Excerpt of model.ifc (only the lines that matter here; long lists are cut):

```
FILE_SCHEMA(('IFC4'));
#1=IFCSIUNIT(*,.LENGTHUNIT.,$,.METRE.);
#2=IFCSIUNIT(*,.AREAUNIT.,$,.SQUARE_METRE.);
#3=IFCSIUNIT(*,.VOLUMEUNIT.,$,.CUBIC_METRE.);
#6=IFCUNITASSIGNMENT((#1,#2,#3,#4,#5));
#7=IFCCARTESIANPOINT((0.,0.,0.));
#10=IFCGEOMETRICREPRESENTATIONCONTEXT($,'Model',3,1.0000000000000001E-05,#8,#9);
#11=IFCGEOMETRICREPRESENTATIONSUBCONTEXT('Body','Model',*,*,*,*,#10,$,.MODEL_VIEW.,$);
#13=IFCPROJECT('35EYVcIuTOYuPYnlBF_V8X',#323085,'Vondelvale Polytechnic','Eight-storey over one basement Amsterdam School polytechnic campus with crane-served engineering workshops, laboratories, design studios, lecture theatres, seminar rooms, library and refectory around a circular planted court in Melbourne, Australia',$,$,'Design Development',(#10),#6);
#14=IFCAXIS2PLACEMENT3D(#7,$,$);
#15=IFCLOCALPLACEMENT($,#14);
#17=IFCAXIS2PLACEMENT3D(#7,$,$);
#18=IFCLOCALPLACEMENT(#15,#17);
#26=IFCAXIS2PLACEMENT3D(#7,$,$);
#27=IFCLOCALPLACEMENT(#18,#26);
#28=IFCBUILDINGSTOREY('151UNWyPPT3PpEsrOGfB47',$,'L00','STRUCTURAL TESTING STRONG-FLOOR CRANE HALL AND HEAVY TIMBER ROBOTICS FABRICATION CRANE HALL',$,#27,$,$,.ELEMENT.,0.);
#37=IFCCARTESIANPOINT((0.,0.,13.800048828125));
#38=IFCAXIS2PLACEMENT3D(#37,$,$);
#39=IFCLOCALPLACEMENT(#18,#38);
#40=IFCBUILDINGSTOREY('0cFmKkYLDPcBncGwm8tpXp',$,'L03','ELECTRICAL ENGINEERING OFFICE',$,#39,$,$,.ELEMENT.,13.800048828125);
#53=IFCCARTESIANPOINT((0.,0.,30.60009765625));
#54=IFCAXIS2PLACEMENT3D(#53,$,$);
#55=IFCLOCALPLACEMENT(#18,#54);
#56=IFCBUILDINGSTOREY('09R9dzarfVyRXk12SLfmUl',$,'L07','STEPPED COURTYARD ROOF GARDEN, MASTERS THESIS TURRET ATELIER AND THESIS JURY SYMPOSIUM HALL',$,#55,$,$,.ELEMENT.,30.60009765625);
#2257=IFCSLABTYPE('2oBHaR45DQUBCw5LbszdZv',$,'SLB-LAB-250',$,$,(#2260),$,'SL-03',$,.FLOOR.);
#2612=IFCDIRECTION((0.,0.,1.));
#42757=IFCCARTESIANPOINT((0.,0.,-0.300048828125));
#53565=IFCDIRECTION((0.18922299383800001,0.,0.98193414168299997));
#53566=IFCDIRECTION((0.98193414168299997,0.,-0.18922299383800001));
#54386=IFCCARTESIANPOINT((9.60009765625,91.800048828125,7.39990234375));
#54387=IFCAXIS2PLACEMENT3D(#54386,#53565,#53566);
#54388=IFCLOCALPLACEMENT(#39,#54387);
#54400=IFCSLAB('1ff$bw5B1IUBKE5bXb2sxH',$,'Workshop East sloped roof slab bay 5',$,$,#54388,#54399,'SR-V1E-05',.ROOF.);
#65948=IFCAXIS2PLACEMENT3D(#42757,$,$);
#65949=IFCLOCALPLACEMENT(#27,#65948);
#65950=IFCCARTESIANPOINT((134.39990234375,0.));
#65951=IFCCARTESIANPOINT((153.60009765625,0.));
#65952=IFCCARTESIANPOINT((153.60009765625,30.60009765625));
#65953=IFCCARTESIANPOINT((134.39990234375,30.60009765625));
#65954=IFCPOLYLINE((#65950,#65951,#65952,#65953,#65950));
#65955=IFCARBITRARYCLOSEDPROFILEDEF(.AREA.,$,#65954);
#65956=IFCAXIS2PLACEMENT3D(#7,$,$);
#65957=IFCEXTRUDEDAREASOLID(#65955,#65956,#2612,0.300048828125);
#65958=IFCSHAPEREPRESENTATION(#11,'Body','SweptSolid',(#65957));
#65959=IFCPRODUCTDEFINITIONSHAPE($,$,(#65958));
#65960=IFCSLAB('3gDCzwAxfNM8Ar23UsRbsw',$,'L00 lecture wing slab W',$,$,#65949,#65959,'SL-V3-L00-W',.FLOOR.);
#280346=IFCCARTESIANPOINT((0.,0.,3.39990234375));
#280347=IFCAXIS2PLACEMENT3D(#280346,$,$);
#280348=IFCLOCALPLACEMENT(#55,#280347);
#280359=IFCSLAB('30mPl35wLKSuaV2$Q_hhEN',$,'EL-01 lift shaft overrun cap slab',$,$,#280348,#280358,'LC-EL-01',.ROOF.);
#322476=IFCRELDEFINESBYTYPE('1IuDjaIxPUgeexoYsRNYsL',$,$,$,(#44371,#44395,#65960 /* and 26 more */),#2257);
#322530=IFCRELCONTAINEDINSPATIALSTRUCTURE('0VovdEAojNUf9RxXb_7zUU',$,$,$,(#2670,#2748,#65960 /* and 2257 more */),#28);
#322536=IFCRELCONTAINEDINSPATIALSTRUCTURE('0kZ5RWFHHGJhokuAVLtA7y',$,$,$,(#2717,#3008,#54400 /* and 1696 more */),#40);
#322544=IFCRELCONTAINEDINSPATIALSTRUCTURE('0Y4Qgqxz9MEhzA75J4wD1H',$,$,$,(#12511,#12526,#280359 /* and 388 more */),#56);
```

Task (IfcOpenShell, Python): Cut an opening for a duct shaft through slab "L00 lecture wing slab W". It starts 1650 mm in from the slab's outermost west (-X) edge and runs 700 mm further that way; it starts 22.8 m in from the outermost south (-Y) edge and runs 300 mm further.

```python
import numpy as np
import ifcopenshell
import ifcopenshell.api.feature
import ifcopenshell.api.geometry
import ifcopenshell.api.root
import ifcopenshell.geom
import ifcopenshell.util.placement
import ifcopenshell.util.representation
import ifcopenshell.util.shape
import ifcopenshell.util.unit

model = ifcopenshell.open("model.ifc")
unit_scale = ifcopenshell.util.unit.calculate_unit_scale(model)
settings = ifcopenshell.geom.settings()


def volume(element):
    """Net volume in cubic metres, openings subtracted."""
    shape = ifcopenshell.geom.create_shape(settings, element)
    return ifcopenshell.util.shape.get_volume(shape.geometry)


slab = model.by_guid("3gDCzwAxfNM8Ar23UsRbsw")
before = volume(slab)

# Extent in the slab's own axes, in metres. The edges named are its -X and -Y sides.
slab_shape = ifcopenshell.geom.create_shape(settings, slab)
vertices = ifcopenshell.util.shape.get_vertices(slab_shape.geometry)
x_min, y_min, bottom = vertices.min(axis=0)
top = vertices[:, 2].max()

opening = ifcopenshell.api.root.create_entity(model, ifc_class="IfcOpeningElement", name="Duct shaft opening", predefined_type="OPENING")
context = ifcopenshell.util.representation.get_context(model, "Model", "Body", "MODEL_VIEW")
width, depth = 0.7, 0.3
outline = [(0.0, 0.0), (width, 0.0), (width, depth), (0.0, depth), (0.0, 0.0)]
# Overshoot both faces by 50 mm so the cut is clean.
shape = ifcopenshell.api.geometry.add_slab_representation(
    model, context=context, depth=top - bottom + 0.1, polyline=outline
)
ifcopenshell.api.geometry.assign_representation(model, product=opening, representation=shape)

matrix = ifcopenshell.util.placement.get_local_placement(slab.ObjectPlacement)
matrix[:, 3] = matrix @ np.append(np.array([x_min + 1.65, y_min + 22.8, bottom - 0.05]) / unit_scale, 1.0)
ifcopenshell.api.geometry.edit_object_placement(model, product=opening, matrix=matrix, is_si=False)
ifcopenshell.api.feature.add_feature(model, feature=opening, element=slab)

after = volume(slab)

print(f"slab volume {before:.3f} -> {after:.3f} m3")

model.write("model_updated.ifc")
```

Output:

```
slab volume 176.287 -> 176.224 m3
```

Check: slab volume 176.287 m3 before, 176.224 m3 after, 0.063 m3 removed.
